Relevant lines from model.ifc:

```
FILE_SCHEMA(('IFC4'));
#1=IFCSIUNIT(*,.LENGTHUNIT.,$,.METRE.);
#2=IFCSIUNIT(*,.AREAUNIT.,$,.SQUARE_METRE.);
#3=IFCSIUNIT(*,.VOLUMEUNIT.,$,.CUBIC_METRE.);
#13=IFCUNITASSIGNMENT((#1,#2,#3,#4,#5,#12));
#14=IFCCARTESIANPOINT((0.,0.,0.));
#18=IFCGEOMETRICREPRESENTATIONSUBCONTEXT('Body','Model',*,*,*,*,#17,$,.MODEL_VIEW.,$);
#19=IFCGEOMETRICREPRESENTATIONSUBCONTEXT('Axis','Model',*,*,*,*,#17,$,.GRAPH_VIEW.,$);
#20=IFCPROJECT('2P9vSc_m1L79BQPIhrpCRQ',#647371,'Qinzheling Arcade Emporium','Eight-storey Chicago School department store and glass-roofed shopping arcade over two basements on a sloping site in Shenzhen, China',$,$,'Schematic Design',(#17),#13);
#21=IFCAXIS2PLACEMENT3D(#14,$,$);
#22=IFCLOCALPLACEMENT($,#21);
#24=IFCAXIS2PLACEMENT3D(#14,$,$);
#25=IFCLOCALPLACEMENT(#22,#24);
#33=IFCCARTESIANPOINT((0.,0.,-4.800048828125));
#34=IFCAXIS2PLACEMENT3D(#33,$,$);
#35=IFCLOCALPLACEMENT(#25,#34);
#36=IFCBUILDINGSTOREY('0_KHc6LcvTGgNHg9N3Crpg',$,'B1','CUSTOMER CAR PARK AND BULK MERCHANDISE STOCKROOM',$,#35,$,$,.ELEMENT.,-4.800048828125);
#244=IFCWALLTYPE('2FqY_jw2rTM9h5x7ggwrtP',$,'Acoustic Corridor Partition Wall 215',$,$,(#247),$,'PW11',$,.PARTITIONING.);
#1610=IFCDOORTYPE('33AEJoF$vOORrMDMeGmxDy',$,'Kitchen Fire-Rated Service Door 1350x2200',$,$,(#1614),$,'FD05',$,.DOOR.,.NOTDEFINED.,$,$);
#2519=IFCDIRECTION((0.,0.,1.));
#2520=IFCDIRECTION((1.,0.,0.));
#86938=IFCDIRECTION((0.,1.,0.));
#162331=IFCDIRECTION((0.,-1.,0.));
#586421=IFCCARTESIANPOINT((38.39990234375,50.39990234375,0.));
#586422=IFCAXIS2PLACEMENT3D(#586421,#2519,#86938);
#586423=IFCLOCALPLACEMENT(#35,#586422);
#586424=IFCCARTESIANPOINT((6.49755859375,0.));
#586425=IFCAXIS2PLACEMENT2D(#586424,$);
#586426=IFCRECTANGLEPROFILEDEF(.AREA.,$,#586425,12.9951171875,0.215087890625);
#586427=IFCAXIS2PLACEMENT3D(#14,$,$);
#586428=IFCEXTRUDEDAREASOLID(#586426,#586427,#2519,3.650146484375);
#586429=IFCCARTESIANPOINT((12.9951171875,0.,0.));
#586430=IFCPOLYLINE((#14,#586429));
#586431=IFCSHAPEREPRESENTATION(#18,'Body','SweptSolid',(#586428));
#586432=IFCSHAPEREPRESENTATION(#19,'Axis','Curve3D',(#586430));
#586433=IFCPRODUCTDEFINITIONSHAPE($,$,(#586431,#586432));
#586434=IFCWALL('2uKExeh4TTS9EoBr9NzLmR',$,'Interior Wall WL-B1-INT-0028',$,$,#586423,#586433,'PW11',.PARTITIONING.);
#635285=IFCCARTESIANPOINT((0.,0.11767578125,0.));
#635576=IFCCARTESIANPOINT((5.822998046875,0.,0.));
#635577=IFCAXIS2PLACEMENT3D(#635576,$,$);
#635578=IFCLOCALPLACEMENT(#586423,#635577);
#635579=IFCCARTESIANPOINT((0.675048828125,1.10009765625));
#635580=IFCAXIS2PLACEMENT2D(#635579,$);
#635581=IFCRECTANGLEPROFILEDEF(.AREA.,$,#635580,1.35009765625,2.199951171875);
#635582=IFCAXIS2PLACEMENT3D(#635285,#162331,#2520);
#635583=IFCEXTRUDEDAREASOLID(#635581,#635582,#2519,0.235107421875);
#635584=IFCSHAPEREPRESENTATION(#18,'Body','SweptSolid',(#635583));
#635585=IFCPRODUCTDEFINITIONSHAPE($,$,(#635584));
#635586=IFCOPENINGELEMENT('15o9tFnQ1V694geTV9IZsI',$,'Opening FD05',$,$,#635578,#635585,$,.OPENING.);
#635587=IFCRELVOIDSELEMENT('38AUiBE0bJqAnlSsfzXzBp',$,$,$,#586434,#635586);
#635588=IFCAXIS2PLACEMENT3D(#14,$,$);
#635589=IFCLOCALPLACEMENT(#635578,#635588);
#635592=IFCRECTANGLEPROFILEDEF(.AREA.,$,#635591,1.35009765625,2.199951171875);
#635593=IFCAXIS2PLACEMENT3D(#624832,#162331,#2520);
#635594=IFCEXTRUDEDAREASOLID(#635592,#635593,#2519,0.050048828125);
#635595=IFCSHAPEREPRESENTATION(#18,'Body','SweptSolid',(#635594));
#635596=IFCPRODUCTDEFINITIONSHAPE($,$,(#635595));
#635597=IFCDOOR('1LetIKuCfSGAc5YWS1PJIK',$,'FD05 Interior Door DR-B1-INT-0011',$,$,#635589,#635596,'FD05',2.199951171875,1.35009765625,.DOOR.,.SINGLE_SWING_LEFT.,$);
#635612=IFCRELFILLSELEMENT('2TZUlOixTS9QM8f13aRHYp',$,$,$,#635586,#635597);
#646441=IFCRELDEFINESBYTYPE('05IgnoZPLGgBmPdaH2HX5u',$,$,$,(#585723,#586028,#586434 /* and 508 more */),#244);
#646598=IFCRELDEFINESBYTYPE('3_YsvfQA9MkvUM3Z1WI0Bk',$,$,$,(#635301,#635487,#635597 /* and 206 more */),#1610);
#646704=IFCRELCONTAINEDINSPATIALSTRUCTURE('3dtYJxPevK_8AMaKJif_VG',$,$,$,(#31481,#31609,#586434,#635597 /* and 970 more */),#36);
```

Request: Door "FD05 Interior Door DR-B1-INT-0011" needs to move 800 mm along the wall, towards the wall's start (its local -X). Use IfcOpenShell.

```python
import ifcopenshell
import ifcopenshell.api.geometry
import ifcopenshell.util.placement
import ifcopenshell.util.unit

model = ifcopenshell.open("model.ifc")
unit_scale = ifcopenshell.util.unit.calculate_unit_scale(model)

door = model.by_guid("1LetIKuCfSGAc5YWS1PJIK")
opening = door.FillsVoids[0].RelatingOpeningElement
wall = opening.VoidsElements[0].RelatingBuildingElement

wall_matrix = ifcopenshell.util.placement.get_local_placement(wall.ObjectPlacement)
shift = wall_matrix[:3, 0] * -0.8 / unit_scale
before = ifcopenshell.util.placement.get_local_placement(door.ObjectPlacement)[:3, 3].copy()

# The door is placed relative to its opening, so it follows when the opening moves.
matrix = ifcopenshell.util.placement.get_local_placement(opening.ObjectPlacement)
matrix[:3, 3] += shift
ifcopenshell.api.geometry.edit_object_placement(
    model, product=opening, matrix=matrix, is_si=False, should_transform_children=True
)

after = ifcopenshell.util.placement.get_local_placement(door.ObjectPlacement)[:3, 3]
print("door moved by", (after - before).round(3) + 0.0)

model.write("model-out.ifc")
```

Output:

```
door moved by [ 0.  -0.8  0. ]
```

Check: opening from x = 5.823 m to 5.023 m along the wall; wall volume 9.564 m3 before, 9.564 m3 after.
